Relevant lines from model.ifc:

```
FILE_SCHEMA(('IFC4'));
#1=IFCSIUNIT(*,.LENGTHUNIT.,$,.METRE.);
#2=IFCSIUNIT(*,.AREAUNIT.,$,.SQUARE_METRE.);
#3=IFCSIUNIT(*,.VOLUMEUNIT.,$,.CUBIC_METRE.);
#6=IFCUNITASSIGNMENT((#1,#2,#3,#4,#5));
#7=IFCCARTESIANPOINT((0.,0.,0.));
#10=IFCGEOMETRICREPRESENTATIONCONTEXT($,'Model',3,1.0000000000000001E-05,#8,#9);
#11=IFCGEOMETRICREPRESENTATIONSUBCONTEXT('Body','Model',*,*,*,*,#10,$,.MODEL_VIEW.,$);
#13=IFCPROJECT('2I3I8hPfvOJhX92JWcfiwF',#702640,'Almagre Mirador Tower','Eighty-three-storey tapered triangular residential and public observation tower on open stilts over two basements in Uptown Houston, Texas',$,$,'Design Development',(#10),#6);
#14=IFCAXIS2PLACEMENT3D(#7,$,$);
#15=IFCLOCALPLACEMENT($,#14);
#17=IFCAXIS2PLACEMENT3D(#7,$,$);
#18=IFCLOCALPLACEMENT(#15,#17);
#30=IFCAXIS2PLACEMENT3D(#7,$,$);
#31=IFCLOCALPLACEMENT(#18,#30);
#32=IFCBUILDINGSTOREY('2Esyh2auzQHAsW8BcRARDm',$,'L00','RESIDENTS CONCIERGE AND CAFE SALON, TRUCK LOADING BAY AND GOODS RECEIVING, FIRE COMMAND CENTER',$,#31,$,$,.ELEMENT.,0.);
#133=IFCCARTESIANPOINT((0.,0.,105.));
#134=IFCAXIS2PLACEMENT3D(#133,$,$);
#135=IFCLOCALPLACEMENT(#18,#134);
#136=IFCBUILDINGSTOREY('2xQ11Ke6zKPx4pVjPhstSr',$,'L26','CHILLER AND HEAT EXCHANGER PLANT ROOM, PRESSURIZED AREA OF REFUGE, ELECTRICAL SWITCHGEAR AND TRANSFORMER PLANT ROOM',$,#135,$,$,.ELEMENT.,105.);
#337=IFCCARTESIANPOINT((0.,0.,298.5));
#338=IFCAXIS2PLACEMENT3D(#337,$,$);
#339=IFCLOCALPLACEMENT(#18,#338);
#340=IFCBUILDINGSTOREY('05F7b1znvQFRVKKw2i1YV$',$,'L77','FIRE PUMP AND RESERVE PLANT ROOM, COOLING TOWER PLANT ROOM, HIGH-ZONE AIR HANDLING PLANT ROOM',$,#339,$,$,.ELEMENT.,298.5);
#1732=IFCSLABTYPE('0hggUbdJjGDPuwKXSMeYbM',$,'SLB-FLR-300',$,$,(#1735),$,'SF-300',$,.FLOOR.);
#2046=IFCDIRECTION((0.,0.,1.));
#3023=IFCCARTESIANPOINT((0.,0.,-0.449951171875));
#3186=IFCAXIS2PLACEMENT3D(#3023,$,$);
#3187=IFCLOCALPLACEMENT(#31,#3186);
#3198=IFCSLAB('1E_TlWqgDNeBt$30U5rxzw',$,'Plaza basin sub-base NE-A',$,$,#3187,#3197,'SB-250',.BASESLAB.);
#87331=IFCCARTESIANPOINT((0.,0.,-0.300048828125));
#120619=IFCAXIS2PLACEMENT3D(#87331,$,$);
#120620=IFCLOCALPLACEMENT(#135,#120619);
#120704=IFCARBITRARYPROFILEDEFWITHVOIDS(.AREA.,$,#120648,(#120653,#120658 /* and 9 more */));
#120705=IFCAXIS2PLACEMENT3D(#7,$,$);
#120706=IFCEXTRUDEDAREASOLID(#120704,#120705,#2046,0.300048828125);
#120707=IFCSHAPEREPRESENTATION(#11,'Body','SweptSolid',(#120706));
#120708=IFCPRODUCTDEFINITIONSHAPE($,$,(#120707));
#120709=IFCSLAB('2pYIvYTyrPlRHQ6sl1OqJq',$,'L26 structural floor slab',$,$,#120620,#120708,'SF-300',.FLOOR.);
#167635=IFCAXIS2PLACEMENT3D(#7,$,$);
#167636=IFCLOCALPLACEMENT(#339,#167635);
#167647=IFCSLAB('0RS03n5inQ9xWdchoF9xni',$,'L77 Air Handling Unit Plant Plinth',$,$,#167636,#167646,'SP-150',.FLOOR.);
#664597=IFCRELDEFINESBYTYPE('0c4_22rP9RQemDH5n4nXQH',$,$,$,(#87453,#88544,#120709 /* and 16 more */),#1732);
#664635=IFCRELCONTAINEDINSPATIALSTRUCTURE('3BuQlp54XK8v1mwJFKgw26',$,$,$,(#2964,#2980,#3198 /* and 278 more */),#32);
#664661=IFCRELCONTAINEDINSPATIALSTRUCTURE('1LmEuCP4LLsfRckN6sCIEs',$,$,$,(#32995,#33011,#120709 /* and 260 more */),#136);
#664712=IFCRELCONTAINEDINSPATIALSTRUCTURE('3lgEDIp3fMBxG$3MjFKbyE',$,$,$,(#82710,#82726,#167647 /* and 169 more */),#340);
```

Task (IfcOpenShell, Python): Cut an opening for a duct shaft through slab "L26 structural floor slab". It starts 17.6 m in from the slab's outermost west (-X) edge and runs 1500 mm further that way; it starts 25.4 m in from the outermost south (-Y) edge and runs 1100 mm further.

```python
import numpy as np
import ifcopenshell
import ifcopenshell.api.feature
import ifcopenshell.api.geometry
import ifcopenshell.api.root
import ifcopenshell.geom
import ifcopenshell.util.placement
import ifcopenshell.util.representation
import ifcopenshell.util.shape
import ifcopenshell.util.unit

model = ifcopenshell.open("model.ifc")
unit_scale = ifcopenshell.util.unit.calculate_unit_scale(model)
settings = ifcopenshell.geom.settings()


def volume(element):
    """Net volume in cubic metres, openings subtracted."""
    shape = ifcopenshell.geom.create_shape(settings, element)
    return ifcopenshell.util.shape.get_volume(shape.geometry)


slab = model.by_guid("2pYIvYTyrPlRHQ6sl1OqJq")
before = volume(slab)

# Extent in the slab's own axes, in metres. The edges named are its -X and -Y sides.
slab_shape = ifcopenshell.geom.create_shape(settings, slab)
vertices = ifcopenshell.util.shape.get_vertices(slab_shape.geometry)
x_min, y_min, bottom = vertices.min(axis=0)
top = vertices[:, 2].max()

opening = ifcopenshell.api.root.create_entity(model, ifc_class="IfcOpeningElement", name="Duct shaft opening", predefined_type="OPENING")
context = ifcopenshell.util.representation.get_context(model, "Model", "Body", "MODEL_VIEW")
width, depth = 1.5, 1.1
outline = [(0.0, 0.0), (width, 0.0), (width, depth), (0.0, depth), (0.0, 0.0)]
# Overshoot both faces by 50 mm so the cut is clean.
shape = ifcopenshell.api.geometry.add_slab_representation(
    model, context=context, depth=top - bottom + 0.1, polyline=outline
)
ifcopenshell.api.geometry.assign_representation(model, product=opening, representation=shape)

matrix = ifcopenshell.util.placement.get_local_placement(slab.ObjectPlacement)
matrix[:, 3] = matrix @ np.append(np.array([x_min + 17.6, y_min + 25.4, bottom - 0.05]) / unit_scale, 1.0)
ifcopenshell.api.geometry.edit_object_placement(model, product=opening, matrix=matrix, is_si=False)
ifcopenshell.api.feature.add_feature(model, feature=opening, element=slab)

after = volume(slab)

print(f"slab volume {before:.3f} -> {after:.3f} m3")

model.write("model_edited.ifc")
```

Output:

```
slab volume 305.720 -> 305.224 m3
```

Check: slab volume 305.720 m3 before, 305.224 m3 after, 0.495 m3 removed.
